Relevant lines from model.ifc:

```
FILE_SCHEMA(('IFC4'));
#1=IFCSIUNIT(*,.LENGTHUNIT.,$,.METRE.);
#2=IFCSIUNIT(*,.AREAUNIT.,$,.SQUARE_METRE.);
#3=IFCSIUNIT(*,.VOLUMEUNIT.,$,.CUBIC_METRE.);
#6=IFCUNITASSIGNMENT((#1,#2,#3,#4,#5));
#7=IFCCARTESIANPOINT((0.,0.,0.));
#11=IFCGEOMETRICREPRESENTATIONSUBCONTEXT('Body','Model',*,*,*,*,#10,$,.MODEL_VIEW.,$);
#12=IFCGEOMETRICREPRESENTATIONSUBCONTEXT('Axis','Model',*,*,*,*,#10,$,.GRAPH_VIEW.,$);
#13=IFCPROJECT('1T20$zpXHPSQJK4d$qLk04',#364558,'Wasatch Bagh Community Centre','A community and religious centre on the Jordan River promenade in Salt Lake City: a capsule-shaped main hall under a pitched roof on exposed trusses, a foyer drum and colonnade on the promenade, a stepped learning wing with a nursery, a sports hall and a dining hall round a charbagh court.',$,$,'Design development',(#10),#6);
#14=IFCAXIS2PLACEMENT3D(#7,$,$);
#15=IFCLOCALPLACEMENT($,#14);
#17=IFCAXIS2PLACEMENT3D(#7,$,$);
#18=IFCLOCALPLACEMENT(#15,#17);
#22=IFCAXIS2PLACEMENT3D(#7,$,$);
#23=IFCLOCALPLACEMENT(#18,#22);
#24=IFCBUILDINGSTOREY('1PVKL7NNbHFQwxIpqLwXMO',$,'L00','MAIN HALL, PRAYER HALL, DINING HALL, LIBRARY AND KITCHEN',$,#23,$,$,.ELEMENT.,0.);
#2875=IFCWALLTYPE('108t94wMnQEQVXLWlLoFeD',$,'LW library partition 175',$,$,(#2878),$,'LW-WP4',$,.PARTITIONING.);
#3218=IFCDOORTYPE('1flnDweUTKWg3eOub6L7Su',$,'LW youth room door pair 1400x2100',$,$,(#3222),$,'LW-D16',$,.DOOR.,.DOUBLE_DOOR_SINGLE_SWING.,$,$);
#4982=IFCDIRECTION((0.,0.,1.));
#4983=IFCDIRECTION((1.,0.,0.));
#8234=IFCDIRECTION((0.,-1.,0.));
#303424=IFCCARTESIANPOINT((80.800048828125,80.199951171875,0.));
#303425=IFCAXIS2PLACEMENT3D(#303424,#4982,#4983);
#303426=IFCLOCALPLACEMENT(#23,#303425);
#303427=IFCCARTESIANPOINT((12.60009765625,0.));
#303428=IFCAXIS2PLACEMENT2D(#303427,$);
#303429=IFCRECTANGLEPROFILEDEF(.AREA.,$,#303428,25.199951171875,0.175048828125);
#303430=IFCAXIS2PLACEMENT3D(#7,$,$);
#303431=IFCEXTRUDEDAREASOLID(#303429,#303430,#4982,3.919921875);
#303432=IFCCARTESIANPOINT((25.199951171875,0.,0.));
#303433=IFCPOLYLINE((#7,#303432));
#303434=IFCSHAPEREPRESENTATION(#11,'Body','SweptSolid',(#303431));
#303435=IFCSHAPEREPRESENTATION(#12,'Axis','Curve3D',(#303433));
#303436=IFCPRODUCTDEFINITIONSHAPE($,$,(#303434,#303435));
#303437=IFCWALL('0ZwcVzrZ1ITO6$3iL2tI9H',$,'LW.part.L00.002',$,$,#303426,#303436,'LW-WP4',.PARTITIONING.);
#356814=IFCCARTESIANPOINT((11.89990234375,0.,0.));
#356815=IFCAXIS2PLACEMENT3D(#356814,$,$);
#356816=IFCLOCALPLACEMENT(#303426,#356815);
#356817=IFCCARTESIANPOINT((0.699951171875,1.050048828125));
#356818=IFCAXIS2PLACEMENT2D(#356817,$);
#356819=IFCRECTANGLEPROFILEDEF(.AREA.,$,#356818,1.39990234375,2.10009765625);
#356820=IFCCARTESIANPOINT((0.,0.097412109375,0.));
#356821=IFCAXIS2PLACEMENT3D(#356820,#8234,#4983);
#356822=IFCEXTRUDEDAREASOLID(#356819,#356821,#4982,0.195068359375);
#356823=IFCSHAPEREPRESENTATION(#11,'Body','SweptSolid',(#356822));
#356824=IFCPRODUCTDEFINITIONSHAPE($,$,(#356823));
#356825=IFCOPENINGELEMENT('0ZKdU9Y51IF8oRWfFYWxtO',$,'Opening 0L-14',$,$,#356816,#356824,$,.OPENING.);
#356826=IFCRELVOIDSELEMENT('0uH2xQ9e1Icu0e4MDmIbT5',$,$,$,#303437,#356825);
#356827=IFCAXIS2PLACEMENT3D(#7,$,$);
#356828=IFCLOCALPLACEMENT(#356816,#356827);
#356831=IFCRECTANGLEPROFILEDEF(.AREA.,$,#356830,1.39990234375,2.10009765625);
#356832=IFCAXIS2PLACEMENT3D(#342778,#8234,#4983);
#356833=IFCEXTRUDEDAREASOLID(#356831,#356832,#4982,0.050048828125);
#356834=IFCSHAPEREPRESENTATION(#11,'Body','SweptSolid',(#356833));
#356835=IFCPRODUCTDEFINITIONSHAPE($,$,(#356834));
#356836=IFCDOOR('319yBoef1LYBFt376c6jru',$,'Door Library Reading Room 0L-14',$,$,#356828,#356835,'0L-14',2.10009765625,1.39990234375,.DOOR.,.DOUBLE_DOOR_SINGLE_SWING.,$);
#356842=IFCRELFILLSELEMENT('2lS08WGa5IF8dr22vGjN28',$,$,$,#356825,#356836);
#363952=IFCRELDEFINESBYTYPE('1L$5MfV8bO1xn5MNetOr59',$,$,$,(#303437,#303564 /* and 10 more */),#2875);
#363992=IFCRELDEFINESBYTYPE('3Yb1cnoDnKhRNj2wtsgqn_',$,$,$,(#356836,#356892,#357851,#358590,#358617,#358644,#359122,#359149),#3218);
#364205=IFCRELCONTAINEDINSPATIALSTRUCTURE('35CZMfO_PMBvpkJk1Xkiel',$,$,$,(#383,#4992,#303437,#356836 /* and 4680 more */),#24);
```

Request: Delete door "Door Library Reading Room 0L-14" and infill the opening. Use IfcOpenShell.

```python
import ifcopenshell
import ifcopenshell.api.feature
import ifcopenshell.api.root
import ifcopenshell.geom
import ifcopenshell.util.shape

model = ifcopenshell.open("model.ifc")
settings = ifcopenshell.geom.settings()


def volume(element):
    """Net volume in cubic metres, openings subtracted."""
    shape = ifcopenshell.geom.create_shape(settings, element)
    return ifcopenshell.util.shape.get_volume(shape.geometry)


door = model.by_guid("319yBoef1LYBFt376c6jru")
opening = door.FillsVoids[0].RelatingOpeningElement
wall = opening.VoidsElements[0].RelatingBuildingElement
before = volume(wall)

ifcopenshell.api.root.remove_product(model, product=door)
ifcopenshell.api.feature.remove_feature(model, feature=opening)

after = volume(wall)

print(f"wall volume {before:.3f} -> {after:.3f} m3")

model.write("model_rev.ifc")
```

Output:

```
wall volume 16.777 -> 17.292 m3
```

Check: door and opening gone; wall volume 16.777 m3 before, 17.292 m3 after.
